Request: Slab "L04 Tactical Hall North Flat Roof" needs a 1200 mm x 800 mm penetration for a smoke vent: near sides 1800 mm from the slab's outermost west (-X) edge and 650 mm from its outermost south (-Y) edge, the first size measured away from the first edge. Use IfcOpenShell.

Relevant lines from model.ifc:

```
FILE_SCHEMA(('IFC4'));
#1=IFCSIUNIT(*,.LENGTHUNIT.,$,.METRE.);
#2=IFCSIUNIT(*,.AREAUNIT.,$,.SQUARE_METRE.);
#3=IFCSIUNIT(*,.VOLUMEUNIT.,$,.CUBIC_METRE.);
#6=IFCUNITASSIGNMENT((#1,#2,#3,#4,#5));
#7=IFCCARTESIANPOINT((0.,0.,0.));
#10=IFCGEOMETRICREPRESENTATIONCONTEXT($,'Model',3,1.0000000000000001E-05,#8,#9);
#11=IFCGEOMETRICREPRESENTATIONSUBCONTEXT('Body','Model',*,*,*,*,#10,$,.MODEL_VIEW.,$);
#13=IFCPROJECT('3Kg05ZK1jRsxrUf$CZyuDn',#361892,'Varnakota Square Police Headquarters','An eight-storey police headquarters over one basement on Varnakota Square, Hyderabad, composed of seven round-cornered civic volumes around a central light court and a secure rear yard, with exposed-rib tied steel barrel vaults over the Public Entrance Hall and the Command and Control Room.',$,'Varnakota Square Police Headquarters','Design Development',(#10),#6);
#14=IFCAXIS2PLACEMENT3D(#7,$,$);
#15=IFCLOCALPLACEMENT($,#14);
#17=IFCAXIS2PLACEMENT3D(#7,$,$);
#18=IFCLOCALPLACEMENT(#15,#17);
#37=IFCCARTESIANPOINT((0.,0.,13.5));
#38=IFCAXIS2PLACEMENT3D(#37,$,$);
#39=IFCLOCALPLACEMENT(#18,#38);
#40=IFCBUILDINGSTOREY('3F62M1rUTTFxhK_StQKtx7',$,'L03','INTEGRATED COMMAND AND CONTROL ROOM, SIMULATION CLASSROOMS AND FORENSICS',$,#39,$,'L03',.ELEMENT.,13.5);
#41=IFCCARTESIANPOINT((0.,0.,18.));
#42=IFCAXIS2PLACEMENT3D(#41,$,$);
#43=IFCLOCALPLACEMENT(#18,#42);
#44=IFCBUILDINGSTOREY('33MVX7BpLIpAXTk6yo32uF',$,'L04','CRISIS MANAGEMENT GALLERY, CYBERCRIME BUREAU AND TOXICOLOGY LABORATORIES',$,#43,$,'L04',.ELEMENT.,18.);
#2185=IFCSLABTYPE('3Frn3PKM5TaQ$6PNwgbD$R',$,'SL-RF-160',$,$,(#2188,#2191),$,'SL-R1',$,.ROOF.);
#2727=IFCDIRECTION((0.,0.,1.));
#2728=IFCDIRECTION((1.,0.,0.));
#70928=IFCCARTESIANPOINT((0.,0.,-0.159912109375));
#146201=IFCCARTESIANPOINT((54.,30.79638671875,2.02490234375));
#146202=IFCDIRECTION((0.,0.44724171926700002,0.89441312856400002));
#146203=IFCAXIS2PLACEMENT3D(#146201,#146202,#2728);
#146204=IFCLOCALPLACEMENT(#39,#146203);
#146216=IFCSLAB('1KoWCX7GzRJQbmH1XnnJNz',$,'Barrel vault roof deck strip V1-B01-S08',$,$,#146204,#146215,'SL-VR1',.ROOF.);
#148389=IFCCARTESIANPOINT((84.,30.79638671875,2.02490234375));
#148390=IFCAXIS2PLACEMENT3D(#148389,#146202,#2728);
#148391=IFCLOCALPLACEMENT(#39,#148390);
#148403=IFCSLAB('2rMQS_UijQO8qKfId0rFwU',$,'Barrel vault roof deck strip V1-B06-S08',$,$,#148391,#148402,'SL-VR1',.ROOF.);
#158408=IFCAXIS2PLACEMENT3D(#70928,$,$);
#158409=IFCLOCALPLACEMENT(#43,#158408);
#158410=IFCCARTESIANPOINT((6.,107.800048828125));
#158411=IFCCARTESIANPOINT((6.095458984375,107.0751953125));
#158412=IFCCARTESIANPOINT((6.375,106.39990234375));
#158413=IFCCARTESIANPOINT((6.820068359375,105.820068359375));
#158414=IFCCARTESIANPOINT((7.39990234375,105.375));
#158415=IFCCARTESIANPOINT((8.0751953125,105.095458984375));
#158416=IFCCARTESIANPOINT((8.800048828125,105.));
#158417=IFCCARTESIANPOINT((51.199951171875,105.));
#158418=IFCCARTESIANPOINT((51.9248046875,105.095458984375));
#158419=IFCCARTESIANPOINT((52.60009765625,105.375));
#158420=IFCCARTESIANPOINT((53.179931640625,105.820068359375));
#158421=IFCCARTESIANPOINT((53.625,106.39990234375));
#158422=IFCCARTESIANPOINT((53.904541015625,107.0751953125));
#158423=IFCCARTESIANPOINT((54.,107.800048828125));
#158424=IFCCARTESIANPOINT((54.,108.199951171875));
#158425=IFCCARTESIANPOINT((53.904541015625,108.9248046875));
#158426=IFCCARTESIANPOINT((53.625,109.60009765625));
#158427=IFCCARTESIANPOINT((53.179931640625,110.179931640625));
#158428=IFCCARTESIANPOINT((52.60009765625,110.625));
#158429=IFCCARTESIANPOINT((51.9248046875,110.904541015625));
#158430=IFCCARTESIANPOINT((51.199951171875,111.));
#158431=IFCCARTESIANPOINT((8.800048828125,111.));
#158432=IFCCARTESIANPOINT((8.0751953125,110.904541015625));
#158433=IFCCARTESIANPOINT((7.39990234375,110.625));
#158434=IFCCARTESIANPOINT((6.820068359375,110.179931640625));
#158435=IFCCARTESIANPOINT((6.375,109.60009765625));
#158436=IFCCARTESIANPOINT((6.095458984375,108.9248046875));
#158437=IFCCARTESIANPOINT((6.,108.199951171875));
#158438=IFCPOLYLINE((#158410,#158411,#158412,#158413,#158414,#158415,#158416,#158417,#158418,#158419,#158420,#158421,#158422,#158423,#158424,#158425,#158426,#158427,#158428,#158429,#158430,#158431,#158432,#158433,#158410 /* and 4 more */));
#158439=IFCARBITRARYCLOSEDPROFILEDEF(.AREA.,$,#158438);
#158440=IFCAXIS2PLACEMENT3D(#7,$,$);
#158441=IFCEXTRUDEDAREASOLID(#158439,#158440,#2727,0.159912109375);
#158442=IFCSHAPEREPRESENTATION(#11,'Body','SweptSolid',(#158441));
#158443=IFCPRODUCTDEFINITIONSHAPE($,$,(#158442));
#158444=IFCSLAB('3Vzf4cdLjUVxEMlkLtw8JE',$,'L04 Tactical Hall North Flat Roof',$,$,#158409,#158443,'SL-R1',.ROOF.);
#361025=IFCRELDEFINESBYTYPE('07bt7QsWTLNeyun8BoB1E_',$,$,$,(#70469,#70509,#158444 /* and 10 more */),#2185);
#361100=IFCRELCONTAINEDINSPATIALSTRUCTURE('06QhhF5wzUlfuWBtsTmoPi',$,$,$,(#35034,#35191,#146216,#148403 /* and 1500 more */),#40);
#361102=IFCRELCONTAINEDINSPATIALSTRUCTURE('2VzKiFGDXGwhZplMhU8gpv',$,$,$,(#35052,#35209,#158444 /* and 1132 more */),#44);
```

```python
import numpy as np
import ifcopenshell
import ifcopenshell.api.feature
import ifcopenshell.api.geometry
import ifcopenshell.api.root
import ifcopenshell.geom
import ifcopenshell.util.placement
import ifcopenshell.util.representation
import ifcopenshell.util.shape
import ifcopenshell.util.unit

model = ifcopenshell.open("model.ifc")
unit_scale = ifcopenshell.util.unit.calculate_unit_scale(model)
settings = ifcopenshell.geom.settings()


def volume(element):
    """Net volume in cubic metres, openings subtracted."""
    shape = ifcopenshell.geom.create_shape(settings, element)
    return ifcopenshell.util.shape.get_volume(shape.geometry)


slab = model.by_id(158444)
before = volume(slab)

# Extent in the slab's own axes, in metres. The edges named are its -X and -Y sides.
slab_shape = ifcopenshell.geom.create_shape(settings, slab)
vertices = ifcopenshell.util.shape.get_vertices(slab_shape.geometry)
x_min, y_min, bottom = vertices.min(axis=0)
top = vertices[:, 2].max()

opening = ifcopenshell.api.root.create_entity(model, ifc_class="IfcOpeningElement", name="Smoke vent opening", predefined_type="OPENING")
context = ifcopenshell.util.representation.get_context(model, "Model", "Body", "MODEL_VIEW")
width, depth = 1.2, 0.8
outline = [(0.0, 0.0), (width, 0.0), (width, depth), (0.0, depth), (0.0, 0.0)]
# Overshoot both faces by 50 mm so the cut is clean.
shape = ifcopenshell.api.geometry.add_slab_representation(
    model, context=context, depth=top - bottom + 0.1, polyline=outline
)
ifcopenshell.api.geometry.assign_representation(model, product=opening, representation=shape)

matrix = ifcopenshell.util.placement.get_local_placement(slab.ObjectPlacement)
matrix[:, 3] = matrix @ np.append(np.array([x_min + 1.8, y_min + 0.65, bottom - 0.05]) / unit_scale, 1.0)
ifcopenshell.api.geometry.edit_object_placement(model, product=opening, matrix=matrix, is_si=False)
ifcopenshell.api.feature.add_feature(model, feature=opening, element=slab)

after = volume(slab)

print(f"slab volume {before:.3f} -> {after:.3f} m3")

model.write("model-out.ifc")
```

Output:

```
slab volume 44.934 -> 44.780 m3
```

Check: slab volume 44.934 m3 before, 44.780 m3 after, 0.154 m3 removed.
